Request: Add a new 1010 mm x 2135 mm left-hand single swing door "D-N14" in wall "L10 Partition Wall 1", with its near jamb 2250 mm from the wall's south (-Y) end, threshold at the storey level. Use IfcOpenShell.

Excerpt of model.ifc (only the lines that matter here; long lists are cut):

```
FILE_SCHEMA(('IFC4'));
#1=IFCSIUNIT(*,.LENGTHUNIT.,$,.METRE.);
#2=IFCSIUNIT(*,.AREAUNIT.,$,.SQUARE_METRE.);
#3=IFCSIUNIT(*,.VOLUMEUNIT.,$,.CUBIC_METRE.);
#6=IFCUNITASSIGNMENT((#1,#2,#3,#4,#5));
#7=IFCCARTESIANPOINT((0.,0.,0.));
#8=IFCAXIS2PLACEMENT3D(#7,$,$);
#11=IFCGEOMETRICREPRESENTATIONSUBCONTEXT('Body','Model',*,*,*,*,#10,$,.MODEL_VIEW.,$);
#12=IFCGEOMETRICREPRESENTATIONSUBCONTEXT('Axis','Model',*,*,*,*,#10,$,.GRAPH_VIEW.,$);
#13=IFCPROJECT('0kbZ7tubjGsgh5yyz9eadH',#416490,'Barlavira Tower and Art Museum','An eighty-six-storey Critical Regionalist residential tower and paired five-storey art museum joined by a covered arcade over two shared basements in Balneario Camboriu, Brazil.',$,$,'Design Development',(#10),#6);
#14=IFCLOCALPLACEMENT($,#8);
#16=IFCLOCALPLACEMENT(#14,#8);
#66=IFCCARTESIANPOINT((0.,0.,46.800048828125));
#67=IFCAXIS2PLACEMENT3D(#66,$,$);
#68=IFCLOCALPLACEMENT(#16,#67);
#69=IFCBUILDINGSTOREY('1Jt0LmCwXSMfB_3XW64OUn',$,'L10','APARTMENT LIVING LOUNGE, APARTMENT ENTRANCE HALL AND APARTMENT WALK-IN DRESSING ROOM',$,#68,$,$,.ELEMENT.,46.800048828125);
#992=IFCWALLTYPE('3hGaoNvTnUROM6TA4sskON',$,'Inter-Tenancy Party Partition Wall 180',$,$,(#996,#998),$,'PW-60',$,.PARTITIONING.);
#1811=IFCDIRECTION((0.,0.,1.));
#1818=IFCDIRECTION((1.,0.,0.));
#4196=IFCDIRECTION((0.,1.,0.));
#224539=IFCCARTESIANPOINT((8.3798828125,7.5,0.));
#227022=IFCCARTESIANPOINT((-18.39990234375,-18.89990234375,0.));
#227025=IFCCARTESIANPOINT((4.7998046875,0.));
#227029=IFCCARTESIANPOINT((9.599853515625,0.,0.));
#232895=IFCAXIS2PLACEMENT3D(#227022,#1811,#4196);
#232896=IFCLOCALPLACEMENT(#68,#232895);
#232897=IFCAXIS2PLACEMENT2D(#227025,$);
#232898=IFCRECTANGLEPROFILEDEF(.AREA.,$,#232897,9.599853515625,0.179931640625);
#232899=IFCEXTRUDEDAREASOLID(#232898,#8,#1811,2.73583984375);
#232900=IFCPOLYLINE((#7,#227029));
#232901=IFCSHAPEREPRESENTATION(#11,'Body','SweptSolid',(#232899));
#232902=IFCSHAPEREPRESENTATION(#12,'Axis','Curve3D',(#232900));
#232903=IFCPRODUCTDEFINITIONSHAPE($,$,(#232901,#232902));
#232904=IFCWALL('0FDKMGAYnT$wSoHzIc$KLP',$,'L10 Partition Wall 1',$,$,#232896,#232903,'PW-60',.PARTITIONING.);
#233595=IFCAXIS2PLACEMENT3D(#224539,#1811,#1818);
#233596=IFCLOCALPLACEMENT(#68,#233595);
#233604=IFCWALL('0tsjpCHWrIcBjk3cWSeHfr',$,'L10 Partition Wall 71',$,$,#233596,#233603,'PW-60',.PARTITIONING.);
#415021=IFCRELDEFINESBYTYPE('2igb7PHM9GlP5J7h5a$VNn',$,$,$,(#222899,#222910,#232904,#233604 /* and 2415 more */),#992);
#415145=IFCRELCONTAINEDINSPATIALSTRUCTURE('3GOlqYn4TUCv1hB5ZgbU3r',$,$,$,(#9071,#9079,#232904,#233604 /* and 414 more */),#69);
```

```python
import numpy as np
import ifcopenshell
import ifcopenshell.api.feature
import ifcopenshell.api.geometry
import ifcopenshell.api.root
import ifcopenshell.api.spatial
import ifcopenshell.geom
import ifcopenshell.util.element
import ifcopenshell.util.placement
import ifcopenshell.util.representation
import ifcopenshell.util.shape
import ifcopenshell.util.unit

model = ifcopenshell.open("model.ifc")
unit_scale = ifcopenshell.util.unit.calculate_unit_scale(model)
settings = ifcopenshell.geom.settings()


def volume(element):
    """Net volume in cubic metres, openings subtracted."""
    shape = ifcopenshell.geom.create_shape(settings, element)
    return ifcopenshell.util.shape.get_volume(shape.geometry)


wall = model.by_id(232904)
storey = ifcopenshell.util.element.get_container(wall, ifc_class="IfcBuildingStorey")
context = ifcopenshell.util.representation.get_context(model, "Model", "Body", "MODEL_VIEW")
before = volume(wall)

width, height, from_end, sill = 1.01, 2.135, 2.25, 0.0  # metres

# The wall runs along its own X axis, and the end named is its -X end.
wall_shape = ifcopenshell.geom.create_shape(settings, wall)
x, y, z = ifcopenshell.util.shape.get_vertices(wall_shape.geometry).T
start = x.min() + from_end
face, thickness = float(y.min()), float(y.max() - y.min())
wall_matrix = ifcopenshell.util.placement.get_local_placement(wall.ObjectPlacement)
level = ifcopenshell.util.placement.get_local_placement(storey.ObjectPlacement)[2, 3]


def in_wall(x, y):
    """Placement at x, y metres in the wall's axes, at sill height."""
    matrix = wall_matrix.copy()
    matrix[:, 3] = wall_matrix @ np.array([x / unit_scale, y / unit_scale, 0.0, 1.0])
    matrix[2, 3] = level + sill / unit_scale
    return matrix


# Opening: a box that overshoots both wall faces by 50 mm.
opening = ifcopenshell.api.root.create_entity(model, ifc_class="IfcOpeningElement", predefined_type="OPENING")
box = ifcopenshell.api.geometry.add_wall_representation(
    model, context=context, length=width, height=height, thickness=thickness + 0.1
)
ifcopenshell.api.geometry.assign_representation(model, product=opening, representation=box)
ifcopenshell.api.geometry.edit_object_placement(model, product=opening, matrix=in_wall(start, face - 0.05), is_si=False)
ifcopenshell.api.feature.add_feature(model, feature=opening, element=wall)

door = ifcopenshell.api.root.create_entity(model, ifc_class="IfcDoor", name="D-N14", predefined_type="DOOR")
door.OverallWidth, door.OverallHeight = width / unit_scale, height / unit_scale
door.OperationType = "SINGLE_SWING_LEFT"
body = ifcopenshell.api.geometry.add_door_representation(
    model,
    context=context,
    overall_width=door.OverallWidth,
    overall_height=door.OverallHeight,
    operation_type="SINGLE_SWING_LEFT",
    lining_properties={"LiningDepth": thickness / unit_scale, "ThresholdDepth": thickness / unit_scale},
)
ifcopenshell.api.geometry.assign_representation(model, product=door, representation=body)
ifcopenshell.api.spatial.assign_container(model, products=[door], relating_structure=storey)
ifcopenshell.api.feature.add_filling(model, opening=opening, element=door)

# The lining spans the wall, so the door starts at the wall face.
ifcopenshell.api.geometry.edit_object_placement(model, product=door, matrix=in_wall(start, face), is_si=False)

after = volume(wall)

print(f"wall volume {before:.3f} -> {after:.3f} m3")

model.write("model_updated.ifc")
```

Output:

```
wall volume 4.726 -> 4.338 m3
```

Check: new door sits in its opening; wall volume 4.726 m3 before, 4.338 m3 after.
